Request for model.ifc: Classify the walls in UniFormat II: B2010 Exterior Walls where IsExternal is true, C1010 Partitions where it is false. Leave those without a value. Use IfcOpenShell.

First a look at what the model holds.

```python
import ifcopenshell
import ifcopenshell.util.element

model = ifcopenshell.open("model.ifc")
print(model.schema)
print("classifications:", [c.Name for c in model.by_type("IfcClassification")])
values = [ifcopenshell.util.element.get_pset(e, "Pset_WallCommon", "IsExternal") for e in model.by_type("IfcWall")]
for value in (True, False, None):
    print("IsExternal", value, values.count(value))
```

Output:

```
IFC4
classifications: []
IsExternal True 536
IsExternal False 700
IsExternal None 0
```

```python
import ifcopenshell
import ifcopenshell.api.classification
import ifcopenshell.util.element

model = ifcopenshell.open("model.ifc")

system = ifcopenshell.api.classification.add_classification(model, classification="UniFormat II")

walls = model.by_type("IfcWall")
external = {e: ifcopenshell.util.element.get_pset(e, "Pset_WallCommon", "IsExternal") for e in walls}
for flag, code, name in ((True, "B2010", "Exterior Walls"), (False, "C1010", "Partitions")):
    products = [e for e in walls if external[e] is flag]
    ifcopenshell.api.classification.add_reference(
        model, products=products, classification=system, identification=code, name=name
    )
    print(code, len(products))

model.write("model-out.ifc")
```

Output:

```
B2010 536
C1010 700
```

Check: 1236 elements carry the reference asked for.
